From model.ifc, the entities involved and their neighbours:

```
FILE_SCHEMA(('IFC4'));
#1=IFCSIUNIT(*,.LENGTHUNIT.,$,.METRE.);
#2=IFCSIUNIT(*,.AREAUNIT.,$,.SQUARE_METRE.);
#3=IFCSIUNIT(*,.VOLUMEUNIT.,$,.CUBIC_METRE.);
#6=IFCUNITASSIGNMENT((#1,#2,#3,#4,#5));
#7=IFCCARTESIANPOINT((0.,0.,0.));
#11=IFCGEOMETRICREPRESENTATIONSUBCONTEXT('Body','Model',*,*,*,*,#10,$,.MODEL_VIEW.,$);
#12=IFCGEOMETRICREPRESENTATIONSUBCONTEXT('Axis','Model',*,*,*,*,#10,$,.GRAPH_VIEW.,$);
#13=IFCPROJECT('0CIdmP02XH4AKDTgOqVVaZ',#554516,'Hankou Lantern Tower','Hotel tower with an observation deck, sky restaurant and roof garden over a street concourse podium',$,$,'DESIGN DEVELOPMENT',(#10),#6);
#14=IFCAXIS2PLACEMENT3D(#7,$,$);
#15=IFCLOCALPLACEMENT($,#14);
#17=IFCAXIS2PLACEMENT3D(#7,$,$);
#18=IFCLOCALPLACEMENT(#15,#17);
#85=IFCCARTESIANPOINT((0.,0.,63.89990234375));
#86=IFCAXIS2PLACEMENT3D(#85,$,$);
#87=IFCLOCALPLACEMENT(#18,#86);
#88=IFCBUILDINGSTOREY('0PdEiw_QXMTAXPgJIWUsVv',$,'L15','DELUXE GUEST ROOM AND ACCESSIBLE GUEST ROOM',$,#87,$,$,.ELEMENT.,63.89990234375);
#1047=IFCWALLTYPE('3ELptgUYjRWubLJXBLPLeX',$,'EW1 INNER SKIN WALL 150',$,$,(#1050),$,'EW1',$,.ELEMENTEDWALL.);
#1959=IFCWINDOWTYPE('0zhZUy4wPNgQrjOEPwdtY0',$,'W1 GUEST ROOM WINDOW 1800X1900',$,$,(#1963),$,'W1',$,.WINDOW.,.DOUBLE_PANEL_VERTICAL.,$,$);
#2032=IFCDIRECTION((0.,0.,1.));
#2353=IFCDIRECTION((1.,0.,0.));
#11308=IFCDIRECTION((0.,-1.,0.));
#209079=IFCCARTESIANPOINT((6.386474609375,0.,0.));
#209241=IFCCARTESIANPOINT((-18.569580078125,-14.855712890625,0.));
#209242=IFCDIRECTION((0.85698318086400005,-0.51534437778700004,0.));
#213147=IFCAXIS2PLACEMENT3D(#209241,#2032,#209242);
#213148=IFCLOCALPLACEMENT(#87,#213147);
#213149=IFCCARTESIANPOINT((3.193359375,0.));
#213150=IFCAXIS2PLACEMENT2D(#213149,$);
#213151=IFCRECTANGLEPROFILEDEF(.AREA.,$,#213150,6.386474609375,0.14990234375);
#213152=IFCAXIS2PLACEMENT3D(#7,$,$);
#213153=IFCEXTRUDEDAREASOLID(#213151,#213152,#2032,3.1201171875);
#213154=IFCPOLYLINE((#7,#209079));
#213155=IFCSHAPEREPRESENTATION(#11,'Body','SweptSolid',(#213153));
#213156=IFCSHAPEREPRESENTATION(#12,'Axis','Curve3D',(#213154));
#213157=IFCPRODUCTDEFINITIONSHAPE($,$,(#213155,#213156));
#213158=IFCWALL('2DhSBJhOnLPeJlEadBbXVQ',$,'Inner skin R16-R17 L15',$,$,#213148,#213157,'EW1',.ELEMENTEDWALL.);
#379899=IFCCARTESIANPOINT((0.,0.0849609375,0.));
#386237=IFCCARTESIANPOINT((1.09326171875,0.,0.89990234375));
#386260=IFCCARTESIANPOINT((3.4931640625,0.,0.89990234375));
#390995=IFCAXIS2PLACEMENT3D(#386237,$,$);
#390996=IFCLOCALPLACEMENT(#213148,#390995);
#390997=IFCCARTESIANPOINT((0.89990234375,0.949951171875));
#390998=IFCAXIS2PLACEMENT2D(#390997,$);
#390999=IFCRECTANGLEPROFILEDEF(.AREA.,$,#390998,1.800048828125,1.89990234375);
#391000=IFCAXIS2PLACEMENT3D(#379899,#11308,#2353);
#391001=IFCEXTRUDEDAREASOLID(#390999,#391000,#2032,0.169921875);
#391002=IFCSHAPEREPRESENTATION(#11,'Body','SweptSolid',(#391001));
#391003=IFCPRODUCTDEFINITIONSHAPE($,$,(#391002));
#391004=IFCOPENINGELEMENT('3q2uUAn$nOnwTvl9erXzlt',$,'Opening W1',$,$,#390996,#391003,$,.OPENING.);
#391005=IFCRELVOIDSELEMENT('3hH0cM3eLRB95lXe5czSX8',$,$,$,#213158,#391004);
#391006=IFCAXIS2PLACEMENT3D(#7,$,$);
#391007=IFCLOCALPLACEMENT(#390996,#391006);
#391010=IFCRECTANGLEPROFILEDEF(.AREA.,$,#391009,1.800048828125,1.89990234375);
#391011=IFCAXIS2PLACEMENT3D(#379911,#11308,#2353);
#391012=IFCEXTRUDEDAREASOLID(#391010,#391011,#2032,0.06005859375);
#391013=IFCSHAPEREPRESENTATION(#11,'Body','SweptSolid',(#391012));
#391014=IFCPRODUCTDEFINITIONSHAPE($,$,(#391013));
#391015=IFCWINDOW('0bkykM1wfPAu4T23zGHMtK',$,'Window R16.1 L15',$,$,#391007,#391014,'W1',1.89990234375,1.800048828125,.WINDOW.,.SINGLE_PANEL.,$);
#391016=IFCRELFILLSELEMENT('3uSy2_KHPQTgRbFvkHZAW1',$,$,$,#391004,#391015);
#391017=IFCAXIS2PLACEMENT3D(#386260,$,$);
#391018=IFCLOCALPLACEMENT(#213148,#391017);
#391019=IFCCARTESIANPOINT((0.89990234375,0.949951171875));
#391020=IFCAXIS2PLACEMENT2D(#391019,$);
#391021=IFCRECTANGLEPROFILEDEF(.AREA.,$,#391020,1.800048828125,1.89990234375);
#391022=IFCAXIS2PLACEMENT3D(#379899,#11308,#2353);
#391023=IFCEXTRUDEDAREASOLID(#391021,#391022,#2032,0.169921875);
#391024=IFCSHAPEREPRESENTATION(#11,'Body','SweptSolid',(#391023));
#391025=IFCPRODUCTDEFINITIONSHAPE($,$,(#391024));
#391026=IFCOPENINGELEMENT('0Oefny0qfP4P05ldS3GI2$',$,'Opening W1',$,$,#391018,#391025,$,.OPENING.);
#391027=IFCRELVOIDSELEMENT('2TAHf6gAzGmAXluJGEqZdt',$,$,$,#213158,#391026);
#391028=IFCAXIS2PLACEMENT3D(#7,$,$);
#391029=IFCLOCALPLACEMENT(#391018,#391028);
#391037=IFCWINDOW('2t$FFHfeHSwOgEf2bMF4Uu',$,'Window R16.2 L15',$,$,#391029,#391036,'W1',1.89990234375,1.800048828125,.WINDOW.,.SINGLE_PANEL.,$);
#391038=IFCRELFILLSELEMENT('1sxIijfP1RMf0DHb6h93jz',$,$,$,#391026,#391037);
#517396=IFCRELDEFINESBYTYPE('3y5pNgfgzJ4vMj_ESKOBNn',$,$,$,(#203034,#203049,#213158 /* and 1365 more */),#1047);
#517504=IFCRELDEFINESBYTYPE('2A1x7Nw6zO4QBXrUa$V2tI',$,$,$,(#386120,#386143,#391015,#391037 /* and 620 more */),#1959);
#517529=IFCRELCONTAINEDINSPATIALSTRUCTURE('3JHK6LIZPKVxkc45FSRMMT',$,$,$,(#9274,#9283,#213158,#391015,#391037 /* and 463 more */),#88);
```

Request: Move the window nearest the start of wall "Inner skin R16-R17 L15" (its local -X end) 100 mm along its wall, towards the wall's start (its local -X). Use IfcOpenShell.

```python
import ifcopenshell
import ifcopenshell.api.geometry
import ifcopenshell.util.placement
import ifcopenshell.util.unit

model = ifcopenshell.open("model.ifc")
unit_scale = ifcopenshell.util.unit.calculate_unit_scale(model)

window = model.by_guid("0bkykM1wfPAu4T23zGHMtK")
opening = window.FillsVoids[0].RelatingOpeningElement
wall = opening.VoidsElements[0].RelatingBuildingElement

wall_matrix = ifcopenshell.util.placement.get_local_placement(wall.ObjectPlacement)
shift = wall_matrix[:3, 0] * -0.1 / unit_scale
before = ifcopenshell.util.placement.get_local_placement(window.ObjectPlacement)[:3, 3].copy()

# The window is placed relative to its opening, so it follows when the opening moves.
matrix = ifcopenshell.util.placement.get_local_placement(opening.ObjectPlacement)
matrix[:3, 3] += shift
ifcopenshell.api.geometry.edit_object_placement(
    model, product=opening, matrix=matrix, is_si=False, should_transform_children=True
)

after = ifcopenshell.util.placement.get_local_placement(window.ObjectPlacement)[:3, 3]
print("window moved by", (after - before).round(3) + 0.0)

model.write("model_rev.ifc")
```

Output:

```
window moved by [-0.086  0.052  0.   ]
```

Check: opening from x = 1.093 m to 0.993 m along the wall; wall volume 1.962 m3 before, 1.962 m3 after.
